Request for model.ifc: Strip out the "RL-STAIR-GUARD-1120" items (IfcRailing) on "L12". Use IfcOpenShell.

First a look at what the model holds.

```python
import ifcopenshell
import ifcopenshell.util.element

model = ifcopenshell.open("model.ifc")
print(model.schema)
storey = next(s for s in model.by_type("IfcBuildingStorey") if s.Name == "L12")
railings = [e for e in ifcopenshell.util.element.get_decomposition(storey) if e.is_a("IfcRailing")]
seen = {}
for e in railings:
    element_type = ifcopenshell.util.element.get_type(e)
    name = element_type.Name if element_type not in (None, e) else None
    seen[name] = seen.get(name, 0) + 1
for name, count in sorted(seen.items(), key=str):
    print(count, "x", name)
```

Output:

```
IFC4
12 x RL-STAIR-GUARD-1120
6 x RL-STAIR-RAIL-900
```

```python
import ifcopenshell
import ifcopenshell.api.root
import ifcopenshell.util.element

model = ifcopenshell.open("model.ifc")

storey = next(s for s in model.by_type("IfcBuildingStorey") if s.Name == "L12")
railings = [e for e in ifcopenshell.util.element.get_decomposition(storey) if e.is_a("IfcRailing")]
targets = [e for e in railings if (t := ifcopenshell.util.element.get_type(e)) not in (None, e) and t.Name == "RL-STAIR-GUARD-1120"]

for e in targets:
    ifcopenshell.api.root.remove_product(model, product=e)
print(len(targets), "removed")

model.write("model-out.ifc")
```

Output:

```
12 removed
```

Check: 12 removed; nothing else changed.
